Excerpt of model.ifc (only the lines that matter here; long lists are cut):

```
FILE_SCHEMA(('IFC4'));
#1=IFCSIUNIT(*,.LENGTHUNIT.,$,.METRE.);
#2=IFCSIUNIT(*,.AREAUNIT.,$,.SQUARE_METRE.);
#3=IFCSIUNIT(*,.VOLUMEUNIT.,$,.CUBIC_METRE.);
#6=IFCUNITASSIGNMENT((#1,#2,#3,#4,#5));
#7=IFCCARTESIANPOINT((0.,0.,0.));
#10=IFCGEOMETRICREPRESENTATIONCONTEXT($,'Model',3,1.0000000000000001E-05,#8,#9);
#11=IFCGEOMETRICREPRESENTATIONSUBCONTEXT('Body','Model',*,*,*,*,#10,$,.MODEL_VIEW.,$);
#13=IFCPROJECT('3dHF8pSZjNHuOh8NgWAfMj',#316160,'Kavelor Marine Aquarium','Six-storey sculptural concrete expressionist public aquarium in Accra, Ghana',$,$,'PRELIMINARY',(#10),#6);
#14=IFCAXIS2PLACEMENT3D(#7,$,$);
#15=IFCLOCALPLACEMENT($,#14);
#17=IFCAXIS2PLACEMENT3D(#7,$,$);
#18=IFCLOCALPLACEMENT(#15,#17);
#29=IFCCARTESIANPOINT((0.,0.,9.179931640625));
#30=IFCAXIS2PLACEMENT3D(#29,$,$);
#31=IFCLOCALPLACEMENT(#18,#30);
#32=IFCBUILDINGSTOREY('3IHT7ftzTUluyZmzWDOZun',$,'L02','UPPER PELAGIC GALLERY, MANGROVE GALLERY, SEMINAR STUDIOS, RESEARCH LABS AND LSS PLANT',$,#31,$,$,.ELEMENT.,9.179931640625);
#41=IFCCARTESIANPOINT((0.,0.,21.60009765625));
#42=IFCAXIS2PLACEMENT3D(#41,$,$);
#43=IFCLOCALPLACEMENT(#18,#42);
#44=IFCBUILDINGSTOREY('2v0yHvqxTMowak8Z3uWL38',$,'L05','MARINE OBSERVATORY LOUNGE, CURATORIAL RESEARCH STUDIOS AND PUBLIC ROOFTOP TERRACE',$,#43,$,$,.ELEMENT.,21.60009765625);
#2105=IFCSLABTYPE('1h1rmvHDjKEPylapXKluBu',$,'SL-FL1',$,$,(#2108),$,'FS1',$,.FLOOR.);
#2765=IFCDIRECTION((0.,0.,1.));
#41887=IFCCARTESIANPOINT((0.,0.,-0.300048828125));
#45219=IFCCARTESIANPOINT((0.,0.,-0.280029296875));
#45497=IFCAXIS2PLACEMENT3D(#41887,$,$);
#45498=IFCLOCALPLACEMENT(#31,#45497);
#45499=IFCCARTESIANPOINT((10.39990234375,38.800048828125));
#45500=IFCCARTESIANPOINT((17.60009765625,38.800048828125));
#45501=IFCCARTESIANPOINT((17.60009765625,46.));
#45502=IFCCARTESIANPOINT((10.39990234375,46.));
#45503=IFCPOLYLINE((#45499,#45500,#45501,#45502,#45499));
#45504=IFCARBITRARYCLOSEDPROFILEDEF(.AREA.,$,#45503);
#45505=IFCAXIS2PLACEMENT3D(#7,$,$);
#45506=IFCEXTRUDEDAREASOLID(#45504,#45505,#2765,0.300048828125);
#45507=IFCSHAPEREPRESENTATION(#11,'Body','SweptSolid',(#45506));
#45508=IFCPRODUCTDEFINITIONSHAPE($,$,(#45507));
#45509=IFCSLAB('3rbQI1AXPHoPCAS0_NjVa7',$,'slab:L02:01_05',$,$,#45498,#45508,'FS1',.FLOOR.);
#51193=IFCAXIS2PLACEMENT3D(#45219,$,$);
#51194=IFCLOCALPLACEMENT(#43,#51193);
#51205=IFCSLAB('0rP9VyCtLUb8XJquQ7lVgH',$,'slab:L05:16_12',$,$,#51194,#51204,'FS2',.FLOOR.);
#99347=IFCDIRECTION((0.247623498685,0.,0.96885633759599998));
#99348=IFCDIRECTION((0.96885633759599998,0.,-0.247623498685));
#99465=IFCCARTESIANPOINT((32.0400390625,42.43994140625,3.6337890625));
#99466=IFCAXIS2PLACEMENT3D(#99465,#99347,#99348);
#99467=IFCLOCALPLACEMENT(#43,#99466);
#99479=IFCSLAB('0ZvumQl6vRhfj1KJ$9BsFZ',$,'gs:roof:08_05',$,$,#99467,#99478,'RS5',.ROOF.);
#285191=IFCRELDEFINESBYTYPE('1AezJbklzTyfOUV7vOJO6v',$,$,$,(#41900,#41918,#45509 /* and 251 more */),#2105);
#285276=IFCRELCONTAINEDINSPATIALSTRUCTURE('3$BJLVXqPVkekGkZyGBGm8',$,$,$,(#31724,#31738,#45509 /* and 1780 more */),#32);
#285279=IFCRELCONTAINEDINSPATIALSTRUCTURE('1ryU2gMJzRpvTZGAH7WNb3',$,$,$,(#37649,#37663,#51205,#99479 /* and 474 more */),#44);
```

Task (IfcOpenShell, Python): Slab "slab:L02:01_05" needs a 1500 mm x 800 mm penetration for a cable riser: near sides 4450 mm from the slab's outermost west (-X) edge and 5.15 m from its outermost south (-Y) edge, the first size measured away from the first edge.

```python
import numpy as np
import ifcopenshell
import ifcopenshell.api.feature
import ifcopenshell.api.geometry
import ifcopenshell.api.root
import ifcopenshell.geom
import ifcopenshell.util.placement
import ifcopenshell.util.representation
import ifcopenshell.util.shape
import ifcopenshell.util.unit

model = ifcopenshell.open("model.ifc")
unit_scale = ifcopenshell.util.unit.calculate_unit_scale(model)
settings = ifcopenshell.geom.settings()


def volume(element):
    """Net volume in cubic metres, openings subtracted."""
    shape = ifcopenshell.geom.create_shape(settings, element)
    return ifcopenshell.util.shape.get_volume(shape.geometry)


slab = model.by_guid("3rbQI1AXPHoPCAS0_NjVa7")
before = volume(slab)

# Extent in the slab's own axes, in metres. The edges named are its -X and -Y sides.
slab_shape = ifcopenshell.geom.create_shape(settings, slab)
vertices = ifcopenshell.util.shape.get_vertices(slab_shape.geometry)
x_min, y_min, bottom = vertices.min(axis=0)
top = vertices[:, 2].max()

opening = ifcopenshell.api.root.create_entity(model, ifc_class="IfcOpeningElement", name="Cable riser opening", predefined_type="OPENING")
context = ifcopenshell.util.representation.get_context(model, "Model", "Body", "MODEL_VIEW")
width, depth = 1.5, 0.8
outline = [(0.0, 0.0), (width, 0.0), (width, depth), (0.0, depth), (0.0, 0.0)]
# Overshoot both faces by 50 mm so the cut is clean.
shape = ifcopenshell.api.geometry.add_slab_representation(
    model, context=context, depth=top - bottom + 0.1, polyline=outline
)
ifcopenshell.api.geometry.assign_representation(model, product=opening, representation=shape)

matrix = ifcopenshell.util.placement.get_local_placement(slab.ObjectPlacement)
matrix[:, 3] = matrix @ np.append(np.array([x_min + 4.45, y_min + 5.15, bottom - 0.05]) / unit_scale, 1.0)
ifcopenshell.api.geometry.edit_object_placement(model, product=opening, matrix=matrix, is_si=False)
ifcopenshell.api.feature.add_feature(model, feature=opening, element=slab)

after = volume(slab)

print(f"slab volume {before:.3f} -> {after:.3f} m3")

model.write("model-out.ifc")
```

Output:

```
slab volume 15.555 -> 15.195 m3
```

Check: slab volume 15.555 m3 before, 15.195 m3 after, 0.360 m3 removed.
